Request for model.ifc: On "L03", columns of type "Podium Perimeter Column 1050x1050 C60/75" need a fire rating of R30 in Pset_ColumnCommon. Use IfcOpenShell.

First a look at what the model holds.

```python
import ifcopenshell
import ifcopenshell.util.element

model = ifcopenshell.open("model.ifc")
print(model.schema)
storey = next(s for s in model.by_type("IfcBuildingStorey") if s.Name == "L03")
columns = [e for e in ifcopenshell.util.element.get_decomposition(storey) if e.is_a("IfcColumn")]
seen = {}
for e in columns:
    element_type = ifcopenshell.util.element.get_type(e)
    key = (element_type.Name if element_type != e and element_type else None, ifcopenshell.util.element.get_pset(e, "Pset_ColumnCommon", "FireRating"))
    seen[key] = seen.get(key, 0) + 1
for (name, value), count in sorted(seen.items(), key=str):
    print(count, "x", name, "|", value)
```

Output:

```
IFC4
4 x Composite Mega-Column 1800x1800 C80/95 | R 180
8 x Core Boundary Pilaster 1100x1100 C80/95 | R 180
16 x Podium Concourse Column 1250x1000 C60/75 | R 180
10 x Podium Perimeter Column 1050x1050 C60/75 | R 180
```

```python
import ifcopenshell
import ifcopenshell.api.pset
import ifcopenshell.util.element

model = ifcopenshell.open("model.ifc")

storey = next(s for s in model.by_type("IfcBuildingStorey") if s.Name == "L03")
columns = [e for e in ifcopenshell.util.element.get_decomposition(storey) if e.is_a("IfcColumn")]

count = 0
for e in columns:
    element_type = ifcopenshell.util.element.get_type(e)
    if element_type in (None, e) or element_type.Name != "Podium Perimeter Column 1050x1050 C60/75":
        continue
    found = ifcopenshell.util.element.get_pset(e, "Pset_ColumnCommon", should_inherit=False)
    if found:
        pset = model.by_id(found["id"])
        if len(ifcopenshell.util.element.get_elements_by_pset(pset)) > 1:
            pset = ifcopenshell.api.pset.unshare_pset(model, products=[e], pset=pset)[0]
    else:
        pset = ifcopenshell.api.pset.add_pset(model, product=e, name="Pset_ColumnCommon")
    ifcopenshell.api.pset.edit_pset(model, pset=pset, properties={"FireRating": "R30"})
    count += 1

print(count, "columns updated")

model.write("model-out.ifc")
```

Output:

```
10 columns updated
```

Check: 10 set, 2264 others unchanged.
